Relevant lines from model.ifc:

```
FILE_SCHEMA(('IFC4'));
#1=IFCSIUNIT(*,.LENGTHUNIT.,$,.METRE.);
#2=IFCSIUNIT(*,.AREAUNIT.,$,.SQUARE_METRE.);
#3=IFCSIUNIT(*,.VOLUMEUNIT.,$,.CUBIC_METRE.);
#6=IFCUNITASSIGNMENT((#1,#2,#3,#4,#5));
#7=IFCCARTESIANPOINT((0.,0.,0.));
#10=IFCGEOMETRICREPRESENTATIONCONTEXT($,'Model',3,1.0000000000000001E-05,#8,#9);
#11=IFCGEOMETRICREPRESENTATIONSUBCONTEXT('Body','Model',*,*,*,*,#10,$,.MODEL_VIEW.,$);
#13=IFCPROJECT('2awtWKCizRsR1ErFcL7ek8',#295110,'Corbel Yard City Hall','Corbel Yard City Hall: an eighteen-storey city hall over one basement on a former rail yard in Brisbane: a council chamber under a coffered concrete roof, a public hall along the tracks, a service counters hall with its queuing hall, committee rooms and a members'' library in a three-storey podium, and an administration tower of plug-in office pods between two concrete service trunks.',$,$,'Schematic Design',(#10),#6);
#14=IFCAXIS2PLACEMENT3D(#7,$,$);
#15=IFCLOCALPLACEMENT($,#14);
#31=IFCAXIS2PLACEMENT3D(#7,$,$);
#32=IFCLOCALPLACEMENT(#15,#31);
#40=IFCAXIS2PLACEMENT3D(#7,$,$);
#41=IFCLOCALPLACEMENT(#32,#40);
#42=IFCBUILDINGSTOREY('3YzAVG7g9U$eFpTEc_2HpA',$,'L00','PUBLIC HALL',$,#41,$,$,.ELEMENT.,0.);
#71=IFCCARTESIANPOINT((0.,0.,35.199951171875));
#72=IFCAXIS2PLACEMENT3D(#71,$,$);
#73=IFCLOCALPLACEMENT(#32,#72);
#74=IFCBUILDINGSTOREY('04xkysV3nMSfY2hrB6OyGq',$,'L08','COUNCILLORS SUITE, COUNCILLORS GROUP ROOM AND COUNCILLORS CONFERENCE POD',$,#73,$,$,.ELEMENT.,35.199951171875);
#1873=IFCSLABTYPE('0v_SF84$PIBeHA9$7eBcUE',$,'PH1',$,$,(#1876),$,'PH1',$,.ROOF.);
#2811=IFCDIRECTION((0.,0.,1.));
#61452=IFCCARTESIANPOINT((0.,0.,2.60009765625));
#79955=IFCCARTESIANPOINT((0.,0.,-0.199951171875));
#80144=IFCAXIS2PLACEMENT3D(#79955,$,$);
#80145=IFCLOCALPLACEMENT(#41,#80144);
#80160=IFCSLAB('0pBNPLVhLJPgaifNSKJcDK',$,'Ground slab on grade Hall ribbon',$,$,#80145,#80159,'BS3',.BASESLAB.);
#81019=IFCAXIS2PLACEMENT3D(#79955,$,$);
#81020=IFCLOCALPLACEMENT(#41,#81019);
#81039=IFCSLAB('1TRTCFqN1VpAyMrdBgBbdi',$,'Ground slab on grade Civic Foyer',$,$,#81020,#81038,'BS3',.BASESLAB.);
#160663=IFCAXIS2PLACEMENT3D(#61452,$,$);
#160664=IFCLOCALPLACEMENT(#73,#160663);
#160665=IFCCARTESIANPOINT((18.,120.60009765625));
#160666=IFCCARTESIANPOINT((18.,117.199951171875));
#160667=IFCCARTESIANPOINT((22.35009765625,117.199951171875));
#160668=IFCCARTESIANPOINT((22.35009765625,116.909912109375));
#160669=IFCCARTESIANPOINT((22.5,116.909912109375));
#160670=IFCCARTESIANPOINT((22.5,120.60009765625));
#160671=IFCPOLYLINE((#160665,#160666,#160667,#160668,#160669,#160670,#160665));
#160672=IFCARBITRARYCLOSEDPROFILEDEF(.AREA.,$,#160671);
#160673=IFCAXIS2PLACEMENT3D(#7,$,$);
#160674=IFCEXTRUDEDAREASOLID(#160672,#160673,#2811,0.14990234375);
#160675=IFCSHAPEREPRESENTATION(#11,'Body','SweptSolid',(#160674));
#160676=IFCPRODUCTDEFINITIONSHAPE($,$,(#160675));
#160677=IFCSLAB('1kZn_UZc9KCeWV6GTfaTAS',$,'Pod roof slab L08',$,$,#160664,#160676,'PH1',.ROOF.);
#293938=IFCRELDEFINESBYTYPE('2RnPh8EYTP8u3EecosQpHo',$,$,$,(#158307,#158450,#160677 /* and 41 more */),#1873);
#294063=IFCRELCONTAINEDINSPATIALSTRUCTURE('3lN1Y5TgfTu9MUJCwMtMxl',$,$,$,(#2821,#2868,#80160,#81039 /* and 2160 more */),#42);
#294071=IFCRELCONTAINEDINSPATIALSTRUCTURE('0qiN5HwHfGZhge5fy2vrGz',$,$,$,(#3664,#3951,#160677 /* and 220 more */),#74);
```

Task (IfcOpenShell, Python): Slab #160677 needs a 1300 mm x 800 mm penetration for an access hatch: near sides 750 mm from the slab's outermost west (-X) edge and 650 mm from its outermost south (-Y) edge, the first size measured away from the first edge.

```python
import numpy as np
import ifcopenshell
import ifcopenshell.api.feature
import ifcopenshell.api.geometry
import ifcopenshell.api.root
import ifcopenshell.geom
import ifcopenshell.util.placement
import ifcopenshell.util.representation
import ifcopenshell.util.shape
import ifcopenshell.util.unit

model = ifcopenshell.open("model.ifc")
unit_scale = ifcopenshell.util.unit.calculate_unit_scale(model)
settings = ifcopenshell.geom.settings()


def volume(element):
    """Net volume in cubic metres, openings subtracted."""
    shape = ifcopenshell.geom.create_shape(settings, element)
    return ifcopenshell.util.shape.get_volume(shape.geometry)


slab = model.by_guid("1kZn_UZc9KCeWV6GTfaTAS")
before = volume(slab)

# Extent in the slab's own axes, in metres. The edges named are its -X and -Y sides.
slab_shape = ifcopenshell.geom.create_shape(settings, slab)
vertices = ifcopenshell.util.shape.get_vertices(slab_shape.geometry)
x_min, y_min, bottom = vertices.min(axis=0)
top = vertices[:, 2].max()

opening = ifcopenshell.api.root.create_entity(model, ifc_class="IfcOpeningElement", name="Access hatch opening", predefined_type="OPENING")
context = ifcopenshell.util.representation.get_context(model, "Model", "Body", "MODEL_VIEW")
width, depth = 1.3, 0.8
outline = [(0.0, 0.0), (width, 0.0), (width, depth), (0.0, depth), (0.0, 0.0)]
# Overshoot both faces by 50 mm so the cut is clean.
shape = ifcopenshell.api.geometry.add_slab_representation(
    model, context=context, depth=top - bottom + 0.1, polyline=outline
)
ifcopenshell.api.geometry.assign_representation(model, product=opening, representation=shape)

matrix = ifcopenshell.util.placement.get_local_placement(slab.ObjectPlacement)
matrix[:, 3] = matrix @ np.append(np.array([x_min + 0.75, y_min + 0.65, bottom - 0.05]) / unit_scale, 1.0)
ifcopenshell.api.geometry.edit_object_placement(model, product=opening, matrix=matrix, is_si=False)
ifcopenshell.api.feature.add_feature(model, feature=opening, element=slab)

after = volume(slab)

print(f"slab volume {before:.3f} -> {after:.3f} m3")

model.write("model_updated.ifc")
```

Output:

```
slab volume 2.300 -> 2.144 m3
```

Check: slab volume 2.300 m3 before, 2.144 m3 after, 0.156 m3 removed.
